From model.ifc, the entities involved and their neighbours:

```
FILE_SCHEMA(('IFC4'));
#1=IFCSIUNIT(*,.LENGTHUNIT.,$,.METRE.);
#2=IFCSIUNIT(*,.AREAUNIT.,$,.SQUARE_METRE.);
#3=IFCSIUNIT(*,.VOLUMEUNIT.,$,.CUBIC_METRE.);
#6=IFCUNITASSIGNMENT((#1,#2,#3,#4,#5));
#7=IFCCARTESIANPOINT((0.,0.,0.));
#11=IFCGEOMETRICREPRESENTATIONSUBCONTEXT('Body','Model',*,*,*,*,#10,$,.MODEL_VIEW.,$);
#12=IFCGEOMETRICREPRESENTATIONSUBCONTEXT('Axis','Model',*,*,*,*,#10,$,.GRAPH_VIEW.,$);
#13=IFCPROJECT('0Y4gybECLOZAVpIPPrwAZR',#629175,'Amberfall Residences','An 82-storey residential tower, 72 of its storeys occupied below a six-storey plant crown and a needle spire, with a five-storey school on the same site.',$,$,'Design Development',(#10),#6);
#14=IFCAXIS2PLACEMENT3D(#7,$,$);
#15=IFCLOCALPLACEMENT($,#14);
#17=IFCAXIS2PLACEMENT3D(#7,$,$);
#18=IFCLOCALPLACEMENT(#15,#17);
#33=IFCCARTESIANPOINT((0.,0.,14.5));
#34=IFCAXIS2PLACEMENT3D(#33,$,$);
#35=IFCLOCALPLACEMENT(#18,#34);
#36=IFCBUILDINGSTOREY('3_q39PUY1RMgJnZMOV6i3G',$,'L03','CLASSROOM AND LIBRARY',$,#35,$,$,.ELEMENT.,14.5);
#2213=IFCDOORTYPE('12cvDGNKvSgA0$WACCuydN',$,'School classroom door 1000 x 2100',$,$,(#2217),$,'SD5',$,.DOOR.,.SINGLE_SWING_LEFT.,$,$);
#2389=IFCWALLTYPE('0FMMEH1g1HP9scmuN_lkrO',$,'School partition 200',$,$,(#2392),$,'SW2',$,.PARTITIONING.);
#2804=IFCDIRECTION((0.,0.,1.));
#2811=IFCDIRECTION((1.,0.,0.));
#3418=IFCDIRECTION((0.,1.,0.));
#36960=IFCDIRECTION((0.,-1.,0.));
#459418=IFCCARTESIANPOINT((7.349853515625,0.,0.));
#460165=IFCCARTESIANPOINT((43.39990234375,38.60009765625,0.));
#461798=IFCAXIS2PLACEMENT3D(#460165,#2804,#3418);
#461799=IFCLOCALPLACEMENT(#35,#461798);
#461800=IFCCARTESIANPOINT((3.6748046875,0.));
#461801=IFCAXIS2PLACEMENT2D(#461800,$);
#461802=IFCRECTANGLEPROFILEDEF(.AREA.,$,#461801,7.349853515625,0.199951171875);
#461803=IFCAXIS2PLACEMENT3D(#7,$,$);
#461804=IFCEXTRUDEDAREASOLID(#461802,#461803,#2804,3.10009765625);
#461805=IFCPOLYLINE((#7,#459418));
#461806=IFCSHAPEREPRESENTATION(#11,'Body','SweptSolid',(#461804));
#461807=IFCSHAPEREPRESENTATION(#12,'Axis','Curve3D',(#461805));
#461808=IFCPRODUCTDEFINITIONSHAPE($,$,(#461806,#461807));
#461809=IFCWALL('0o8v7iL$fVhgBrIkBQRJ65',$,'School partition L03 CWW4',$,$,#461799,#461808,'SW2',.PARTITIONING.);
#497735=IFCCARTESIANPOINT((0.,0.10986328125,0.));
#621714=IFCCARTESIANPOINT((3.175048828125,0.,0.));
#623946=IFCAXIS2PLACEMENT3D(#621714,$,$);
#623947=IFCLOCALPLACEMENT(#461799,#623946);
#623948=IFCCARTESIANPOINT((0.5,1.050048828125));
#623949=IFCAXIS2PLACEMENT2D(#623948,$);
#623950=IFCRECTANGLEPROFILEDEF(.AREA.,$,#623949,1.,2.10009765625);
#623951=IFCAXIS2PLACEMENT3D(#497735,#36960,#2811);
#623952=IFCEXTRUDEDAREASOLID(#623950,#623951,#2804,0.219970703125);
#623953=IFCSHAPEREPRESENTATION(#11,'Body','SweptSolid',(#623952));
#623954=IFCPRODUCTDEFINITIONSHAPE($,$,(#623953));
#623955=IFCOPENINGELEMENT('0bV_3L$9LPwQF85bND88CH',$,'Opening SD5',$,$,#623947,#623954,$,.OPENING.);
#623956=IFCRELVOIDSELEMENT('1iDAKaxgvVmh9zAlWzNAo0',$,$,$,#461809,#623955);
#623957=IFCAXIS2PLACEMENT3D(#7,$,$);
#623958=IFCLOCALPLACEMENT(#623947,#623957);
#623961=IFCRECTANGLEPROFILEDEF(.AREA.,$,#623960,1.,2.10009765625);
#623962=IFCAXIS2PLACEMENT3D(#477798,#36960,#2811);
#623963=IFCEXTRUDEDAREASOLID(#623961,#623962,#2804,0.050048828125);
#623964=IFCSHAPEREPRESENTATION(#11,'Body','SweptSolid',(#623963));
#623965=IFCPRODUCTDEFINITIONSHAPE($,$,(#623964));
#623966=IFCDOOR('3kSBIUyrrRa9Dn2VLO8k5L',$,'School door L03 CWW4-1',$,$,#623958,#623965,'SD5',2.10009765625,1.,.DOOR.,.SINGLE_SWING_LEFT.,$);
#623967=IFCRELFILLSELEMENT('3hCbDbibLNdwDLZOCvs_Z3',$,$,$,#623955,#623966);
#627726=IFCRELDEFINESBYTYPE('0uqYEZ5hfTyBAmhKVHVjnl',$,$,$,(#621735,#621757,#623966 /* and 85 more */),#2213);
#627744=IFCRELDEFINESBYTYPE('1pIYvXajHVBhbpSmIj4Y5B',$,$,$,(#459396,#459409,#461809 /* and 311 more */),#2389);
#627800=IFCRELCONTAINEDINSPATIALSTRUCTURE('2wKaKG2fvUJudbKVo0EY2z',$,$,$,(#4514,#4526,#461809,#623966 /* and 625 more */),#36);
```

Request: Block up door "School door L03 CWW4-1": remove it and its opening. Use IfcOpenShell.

```python
import ifcopenshell
import ifcopenshell.api.feature
import ifcopenshell.api.root
import ifcopenshell.geom
import ifcopenshell.util.shape

model = ifcopenshell.open("model.ifc")
settings = ifcopenshell.geom.settings()


def volume(element):
    """Net volume in cubic metres, openings subtracted."""
    shape = ifcopenshell.geom.create_shape(settings, element)
    return ifcopenshell.util.shape.get_volume(shape.geometry)


door = model.by_guid("3kSBIUyrrRa9Dn2VLO8k5L")
opening = door.FillsVoids[0].RelatingOpeningElement
wall = opening.VoidsElements[0].RelatingBuildingElement
before = volume(wall)

ifcopenshell.api.root.remove_product(model, product=door)
ifcopenshell.api.feature.remove_feature(model, feature=opening)

after = volume(wall)

print(f"wall volume {before:.3f} -> {after:.3f} m3")

model.write("model_edited.ifc")
```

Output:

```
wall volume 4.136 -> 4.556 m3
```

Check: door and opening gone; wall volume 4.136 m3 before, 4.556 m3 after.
